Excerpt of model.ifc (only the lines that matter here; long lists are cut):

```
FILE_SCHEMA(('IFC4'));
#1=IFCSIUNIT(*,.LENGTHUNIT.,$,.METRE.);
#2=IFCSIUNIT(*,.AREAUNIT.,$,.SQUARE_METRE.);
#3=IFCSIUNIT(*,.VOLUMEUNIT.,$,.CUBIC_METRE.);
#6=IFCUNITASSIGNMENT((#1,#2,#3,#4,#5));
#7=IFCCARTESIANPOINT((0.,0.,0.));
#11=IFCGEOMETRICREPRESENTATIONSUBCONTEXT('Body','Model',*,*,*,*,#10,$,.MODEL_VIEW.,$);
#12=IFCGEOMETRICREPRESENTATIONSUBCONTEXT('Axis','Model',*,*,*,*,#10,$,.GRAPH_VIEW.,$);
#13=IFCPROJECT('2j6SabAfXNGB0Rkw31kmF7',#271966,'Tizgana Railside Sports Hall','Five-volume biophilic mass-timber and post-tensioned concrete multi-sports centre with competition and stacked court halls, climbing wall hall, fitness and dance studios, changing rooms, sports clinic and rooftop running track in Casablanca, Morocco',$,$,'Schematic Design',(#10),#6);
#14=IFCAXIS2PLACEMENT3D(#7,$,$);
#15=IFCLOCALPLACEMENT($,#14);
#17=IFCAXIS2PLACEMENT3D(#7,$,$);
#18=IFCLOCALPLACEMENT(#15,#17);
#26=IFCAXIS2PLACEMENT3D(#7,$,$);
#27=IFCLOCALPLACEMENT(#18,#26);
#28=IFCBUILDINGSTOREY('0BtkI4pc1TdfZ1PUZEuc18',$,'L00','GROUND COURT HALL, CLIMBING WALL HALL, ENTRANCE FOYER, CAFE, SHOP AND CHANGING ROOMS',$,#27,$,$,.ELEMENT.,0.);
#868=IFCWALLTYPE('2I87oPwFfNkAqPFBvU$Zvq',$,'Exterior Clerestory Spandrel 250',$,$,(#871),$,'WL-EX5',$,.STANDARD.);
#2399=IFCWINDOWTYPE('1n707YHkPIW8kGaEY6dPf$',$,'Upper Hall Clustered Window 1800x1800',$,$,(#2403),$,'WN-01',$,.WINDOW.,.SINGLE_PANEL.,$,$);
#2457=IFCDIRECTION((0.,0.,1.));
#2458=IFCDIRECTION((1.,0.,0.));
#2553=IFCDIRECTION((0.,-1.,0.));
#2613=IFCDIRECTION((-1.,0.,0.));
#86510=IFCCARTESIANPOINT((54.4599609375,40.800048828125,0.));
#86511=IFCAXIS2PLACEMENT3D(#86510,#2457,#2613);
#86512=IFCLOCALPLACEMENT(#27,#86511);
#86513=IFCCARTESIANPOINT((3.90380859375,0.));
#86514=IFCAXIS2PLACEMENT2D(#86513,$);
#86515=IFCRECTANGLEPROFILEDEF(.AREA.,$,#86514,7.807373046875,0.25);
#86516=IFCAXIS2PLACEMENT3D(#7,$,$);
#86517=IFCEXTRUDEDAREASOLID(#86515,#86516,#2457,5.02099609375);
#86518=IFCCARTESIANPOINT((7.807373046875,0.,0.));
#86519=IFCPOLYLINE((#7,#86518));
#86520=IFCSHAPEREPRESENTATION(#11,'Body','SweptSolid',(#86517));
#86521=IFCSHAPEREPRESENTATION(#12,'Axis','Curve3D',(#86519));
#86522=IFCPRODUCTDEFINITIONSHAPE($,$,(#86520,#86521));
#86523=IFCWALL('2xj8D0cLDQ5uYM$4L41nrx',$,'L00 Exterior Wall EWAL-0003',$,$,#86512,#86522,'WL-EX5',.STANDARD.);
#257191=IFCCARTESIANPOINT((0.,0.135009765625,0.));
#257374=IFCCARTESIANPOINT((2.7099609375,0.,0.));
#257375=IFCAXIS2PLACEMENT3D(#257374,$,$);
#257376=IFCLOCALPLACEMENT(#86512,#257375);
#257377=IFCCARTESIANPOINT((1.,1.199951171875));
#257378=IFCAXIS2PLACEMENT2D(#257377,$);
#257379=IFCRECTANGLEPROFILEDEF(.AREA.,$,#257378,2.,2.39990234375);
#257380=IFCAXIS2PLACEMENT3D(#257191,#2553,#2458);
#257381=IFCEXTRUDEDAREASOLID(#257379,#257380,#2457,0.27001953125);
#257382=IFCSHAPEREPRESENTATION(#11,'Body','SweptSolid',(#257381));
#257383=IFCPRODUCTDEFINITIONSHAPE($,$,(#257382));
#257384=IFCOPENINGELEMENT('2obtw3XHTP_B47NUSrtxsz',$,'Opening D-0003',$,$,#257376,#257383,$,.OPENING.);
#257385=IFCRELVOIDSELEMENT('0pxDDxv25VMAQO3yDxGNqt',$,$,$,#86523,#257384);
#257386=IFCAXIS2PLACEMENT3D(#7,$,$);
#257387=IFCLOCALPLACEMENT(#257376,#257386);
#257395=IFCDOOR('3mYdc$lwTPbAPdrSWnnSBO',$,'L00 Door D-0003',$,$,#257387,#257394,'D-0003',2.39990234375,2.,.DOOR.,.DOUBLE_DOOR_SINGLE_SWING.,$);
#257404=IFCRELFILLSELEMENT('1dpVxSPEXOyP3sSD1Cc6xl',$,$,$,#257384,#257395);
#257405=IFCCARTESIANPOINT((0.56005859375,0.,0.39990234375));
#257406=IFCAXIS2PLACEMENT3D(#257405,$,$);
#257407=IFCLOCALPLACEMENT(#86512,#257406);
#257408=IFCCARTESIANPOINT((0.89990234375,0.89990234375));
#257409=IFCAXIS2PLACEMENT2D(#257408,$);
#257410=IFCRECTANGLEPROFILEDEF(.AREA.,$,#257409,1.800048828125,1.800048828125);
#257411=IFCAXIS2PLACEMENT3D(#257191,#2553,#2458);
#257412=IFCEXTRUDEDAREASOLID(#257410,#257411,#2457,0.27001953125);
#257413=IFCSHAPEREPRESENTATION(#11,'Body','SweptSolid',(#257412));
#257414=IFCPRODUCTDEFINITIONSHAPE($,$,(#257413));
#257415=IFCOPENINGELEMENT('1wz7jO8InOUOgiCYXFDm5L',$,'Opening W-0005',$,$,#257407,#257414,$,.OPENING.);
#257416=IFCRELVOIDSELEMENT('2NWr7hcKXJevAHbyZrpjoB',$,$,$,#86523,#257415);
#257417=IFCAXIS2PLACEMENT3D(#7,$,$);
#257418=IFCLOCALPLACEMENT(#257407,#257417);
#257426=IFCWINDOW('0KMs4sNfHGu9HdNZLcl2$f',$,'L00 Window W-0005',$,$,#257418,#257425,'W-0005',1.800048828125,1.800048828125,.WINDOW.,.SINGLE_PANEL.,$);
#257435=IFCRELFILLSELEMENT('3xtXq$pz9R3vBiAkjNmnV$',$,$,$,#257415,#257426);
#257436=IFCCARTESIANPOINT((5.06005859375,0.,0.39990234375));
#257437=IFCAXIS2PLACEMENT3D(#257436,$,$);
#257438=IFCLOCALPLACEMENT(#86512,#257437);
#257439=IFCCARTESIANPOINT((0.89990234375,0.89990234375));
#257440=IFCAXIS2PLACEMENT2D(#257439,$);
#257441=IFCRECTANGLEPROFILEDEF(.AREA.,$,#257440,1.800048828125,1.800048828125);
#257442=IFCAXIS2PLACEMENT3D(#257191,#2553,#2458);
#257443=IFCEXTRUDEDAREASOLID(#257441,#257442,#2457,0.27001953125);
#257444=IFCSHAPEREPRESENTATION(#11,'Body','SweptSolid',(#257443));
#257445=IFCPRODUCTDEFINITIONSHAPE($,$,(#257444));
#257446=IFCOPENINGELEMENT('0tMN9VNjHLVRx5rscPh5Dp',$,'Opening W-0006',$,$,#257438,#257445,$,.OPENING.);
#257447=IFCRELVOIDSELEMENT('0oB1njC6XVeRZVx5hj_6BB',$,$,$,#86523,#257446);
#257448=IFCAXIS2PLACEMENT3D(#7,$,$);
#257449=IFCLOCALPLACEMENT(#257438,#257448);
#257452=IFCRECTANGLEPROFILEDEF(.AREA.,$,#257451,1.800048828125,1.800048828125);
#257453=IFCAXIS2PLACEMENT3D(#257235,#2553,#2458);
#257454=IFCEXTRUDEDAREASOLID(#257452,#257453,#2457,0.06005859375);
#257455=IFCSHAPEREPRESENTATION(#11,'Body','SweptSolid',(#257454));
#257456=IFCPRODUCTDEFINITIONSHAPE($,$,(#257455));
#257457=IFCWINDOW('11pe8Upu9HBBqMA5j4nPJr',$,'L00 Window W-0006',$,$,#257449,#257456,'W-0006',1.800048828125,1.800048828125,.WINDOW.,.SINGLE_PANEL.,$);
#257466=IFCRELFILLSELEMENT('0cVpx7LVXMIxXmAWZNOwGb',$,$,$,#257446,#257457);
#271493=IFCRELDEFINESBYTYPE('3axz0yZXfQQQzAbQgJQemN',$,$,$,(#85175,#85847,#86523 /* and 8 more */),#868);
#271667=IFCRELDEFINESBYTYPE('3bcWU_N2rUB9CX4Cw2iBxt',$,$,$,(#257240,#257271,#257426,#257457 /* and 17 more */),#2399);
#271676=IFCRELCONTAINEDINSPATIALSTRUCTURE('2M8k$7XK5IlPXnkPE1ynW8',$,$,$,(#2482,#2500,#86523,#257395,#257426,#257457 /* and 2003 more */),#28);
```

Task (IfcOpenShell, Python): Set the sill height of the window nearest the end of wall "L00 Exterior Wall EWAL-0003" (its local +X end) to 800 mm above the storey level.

```python
import numpy as np
import ifcopenshell
import ifcopenshell.api.geometry
import ifcopenshell.geom
import ifcopenshell.util.element
import ifcopenshell.util.placement
import ifcopenshell.util.shape
import ifcopenshell.util.unit

model = ifcopenshell.open("model.ifc")
unit_scale = ifcopenshell.util.unit.calculate_unit_scale(model)

window = model.by_guid("11pe8Upu9HBBqMA5j4nPJr")
opening = window.FillsVoids[0].RelatingOpeningElement
storey = ifcopenshell.util.element.get_container(window, ifc_class="IfcBuildingStorey")
level = ifcopenshell.util.placement.get_local_placement(storey.ObjectPlacement)[2, 3]

# The opening's origin need not be at the sill, so measure its lowest point.
shape = ifcopenshell.geom.create_shape(ifcopenshell.geom.settings(), opening)
bottom = ifcopenshell.util.shape.get_shape_bottom_elevation(shape, shape.geometry) / unit_scale
dz = level + 0.8 - bottom

shift = np.array([0.0, 0.0, dz])
# The window is placed relative to its opening, so it follows when the opening moves.
matrix = ifcopenshell.util.placement.get_local_placement(opening.ObjectPlacement)
matrix[:3, 3] += shift
ifcopenshell.api.geometry.edit_object_placement(
    model, product=opening, matrix=matrix, is_si=False, should_transform_children=True
)

print(f"moved by {dz * unit_scale:+.3f} m")

model.write("model_v2.ifc")
```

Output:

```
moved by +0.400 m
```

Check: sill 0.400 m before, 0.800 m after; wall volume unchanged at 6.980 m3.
